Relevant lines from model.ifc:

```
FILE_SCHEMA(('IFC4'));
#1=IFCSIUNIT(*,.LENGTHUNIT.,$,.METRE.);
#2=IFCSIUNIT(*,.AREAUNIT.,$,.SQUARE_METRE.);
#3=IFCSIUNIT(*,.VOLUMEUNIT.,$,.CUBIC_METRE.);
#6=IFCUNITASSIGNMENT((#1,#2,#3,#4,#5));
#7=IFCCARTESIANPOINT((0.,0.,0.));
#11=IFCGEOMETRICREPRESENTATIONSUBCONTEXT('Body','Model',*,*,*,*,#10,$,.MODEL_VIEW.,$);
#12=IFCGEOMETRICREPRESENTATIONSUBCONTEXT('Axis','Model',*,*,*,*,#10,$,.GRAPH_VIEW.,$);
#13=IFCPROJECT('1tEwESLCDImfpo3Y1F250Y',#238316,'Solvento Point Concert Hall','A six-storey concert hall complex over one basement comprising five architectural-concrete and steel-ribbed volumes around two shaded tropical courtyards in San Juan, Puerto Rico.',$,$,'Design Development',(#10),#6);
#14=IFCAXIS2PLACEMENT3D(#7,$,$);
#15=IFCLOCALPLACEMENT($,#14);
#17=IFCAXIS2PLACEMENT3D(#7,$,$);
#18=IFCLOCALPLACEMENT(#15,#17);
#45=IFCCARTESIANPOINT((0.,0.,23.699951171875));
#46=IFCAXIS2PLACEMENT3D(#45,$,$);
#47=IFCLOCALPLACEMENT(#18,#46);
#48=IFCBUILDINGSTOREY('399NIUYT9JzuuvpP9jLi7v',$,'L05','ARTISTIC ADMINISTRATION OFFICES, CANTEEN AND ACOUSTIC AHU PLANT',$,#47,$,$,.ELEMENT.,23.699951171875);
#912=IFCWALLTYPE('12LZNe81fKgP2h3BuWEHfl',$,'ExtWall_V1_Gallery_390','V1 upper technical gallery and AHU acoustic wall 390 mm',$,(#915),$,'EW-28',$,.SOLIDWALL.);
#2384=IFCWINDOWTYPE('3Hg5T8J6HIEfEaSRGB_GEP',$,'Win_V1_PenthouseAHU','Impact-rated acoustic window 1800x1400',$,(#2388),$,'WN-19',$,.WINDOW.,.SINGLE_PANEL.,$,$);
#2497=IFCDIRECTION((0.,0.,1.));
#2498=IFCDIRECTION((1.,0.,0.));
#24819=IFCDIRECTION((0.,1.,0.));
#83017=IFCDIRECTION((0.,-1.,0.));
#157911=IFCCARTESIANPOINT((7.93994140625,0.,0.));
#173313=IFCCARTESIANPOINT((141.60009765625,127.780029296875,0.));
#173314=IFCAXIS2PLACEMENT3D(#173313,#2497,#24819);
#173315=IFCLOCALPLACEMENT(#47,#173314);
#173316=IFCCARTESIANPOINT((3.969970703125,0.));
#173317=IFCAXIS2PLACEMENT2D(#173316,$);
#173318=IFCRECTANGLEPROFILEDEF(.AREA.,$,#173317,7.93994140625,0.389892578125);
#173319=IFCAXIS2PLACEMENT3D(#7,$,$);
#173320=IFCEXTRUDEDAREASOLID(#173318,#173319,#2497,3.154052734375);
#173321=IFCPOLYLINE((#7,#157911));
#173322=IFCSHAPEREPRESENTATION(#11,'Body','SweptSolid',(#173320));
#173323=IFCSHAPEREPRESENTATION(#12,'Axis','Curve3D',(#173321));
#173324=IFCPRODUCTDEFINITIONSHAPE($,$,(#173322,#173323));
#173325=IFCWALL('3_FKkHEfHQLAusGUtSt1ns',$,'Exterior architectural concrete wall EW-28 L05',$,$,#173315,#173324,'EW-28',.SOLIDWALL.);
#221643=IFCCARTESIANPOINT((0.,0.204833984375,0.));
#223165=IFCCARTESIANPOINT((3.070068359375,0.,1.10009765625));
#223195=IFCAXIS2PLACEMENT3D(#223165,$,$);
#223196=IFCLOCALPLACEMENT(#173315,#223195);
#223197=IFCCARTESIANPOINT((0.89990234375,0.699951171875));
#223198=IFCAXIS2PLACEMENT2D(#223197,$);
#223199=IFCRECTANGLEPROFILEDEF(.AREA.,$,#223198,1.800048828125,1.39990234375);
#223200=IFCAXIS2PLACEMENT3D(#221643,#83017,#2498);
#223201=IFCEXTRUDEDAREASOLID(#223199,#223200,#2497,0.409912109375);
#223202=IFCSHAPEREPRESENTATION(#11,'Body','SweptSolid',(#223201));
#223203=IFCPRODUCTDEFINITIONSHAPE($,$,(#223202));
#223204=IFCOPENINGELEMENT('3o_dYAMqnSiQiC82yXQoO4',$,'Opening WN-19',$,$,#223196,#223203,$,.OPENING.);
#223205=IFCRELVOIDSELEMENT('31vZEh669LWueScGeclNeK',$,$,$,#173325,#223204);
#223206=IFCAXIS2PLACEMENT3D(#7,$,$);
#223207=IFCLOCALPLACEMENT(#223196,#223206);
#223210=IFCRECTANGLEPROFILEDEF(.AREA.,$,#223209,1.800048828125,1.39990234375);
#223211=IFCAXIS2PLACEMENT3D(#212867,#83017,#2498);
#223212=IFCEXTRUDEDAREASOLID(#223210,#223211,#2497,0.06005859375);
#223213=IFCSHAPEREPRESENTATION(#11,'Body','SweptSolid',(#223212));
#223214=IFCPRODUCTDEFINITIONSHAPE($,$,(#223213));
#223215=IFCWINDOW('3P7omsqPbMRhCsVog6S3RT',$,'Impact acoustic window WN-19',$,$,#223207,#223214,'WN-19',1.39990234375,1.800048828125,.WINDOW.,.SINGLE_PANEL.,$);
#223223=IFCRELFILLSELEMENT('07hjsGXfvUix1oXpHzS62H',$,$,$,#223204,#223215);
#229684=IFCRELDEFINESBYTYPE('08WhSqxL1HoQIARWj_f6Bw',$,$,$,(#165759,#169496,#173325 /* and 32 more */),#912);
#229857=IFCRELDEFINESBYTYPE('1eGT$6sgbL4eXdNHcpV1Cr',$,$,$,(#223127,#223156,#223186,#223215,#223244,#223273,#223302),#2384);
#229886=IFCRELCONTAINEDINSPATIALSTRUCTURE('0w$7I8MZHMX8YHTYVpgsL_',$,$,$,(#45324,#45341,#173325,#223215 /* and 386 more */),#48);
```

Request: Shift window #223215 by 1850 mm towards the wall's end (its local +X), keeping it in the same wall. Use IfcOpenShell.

```python
import ifcopenshell
import ifcopenshell.api.geometry
import ifcopenshell.util.placement
import ifcopenshell.util.unit

model = ifcopenshell.open("model.ifc")
unit_scale = ifcopenshell.util.unit.calculate_unit_scale(model)

window = model.by_guid("3P7omsqPbMRhCsVog6S3RT")
opening = window.FillsVoids[0].RelatingOpeningElement
wall = opening.VoidsElements[0].RelatingBuildingElement

wall_matrix = ifcopenshell.util.placement.get_local_placement(wall.ObjectPlacement)
shift = wall_matrix[:3, 0] * 1.85 / unit_scale
before = ifcopenshell.util.placement.get_local_placement(window.ObjectPlacement)[:3, 3].copy()

# The window is placed relative to its opening, so it follows when the opening moves.
matrix = ifcopenshell.util.placement.get_local_placement(opening.ObjectPlacement)
matrix[:3, 3] += shift
ifcopenshell.api.geometry.edit_object_placement(
    model, product=opening, matrix=matrix, is_si=False, should_transform_children=True
)

after = ifcopenshell.util.placement.get_local_placement(window.ObjectPlacement)[:3, 3]
print("window moved by", (after - before).round(3) + 0.0)

model.write("model_v2.ifc")
```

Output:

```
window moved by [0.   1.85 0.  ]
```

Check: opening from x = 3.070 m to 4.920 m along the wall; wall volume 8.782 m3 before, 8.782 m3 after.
